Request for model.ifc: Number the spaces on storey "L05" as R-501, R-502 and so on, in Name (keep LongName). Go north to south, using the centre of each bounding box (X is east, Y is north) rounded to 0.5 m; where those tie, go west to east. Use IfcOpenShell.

First a look at what the model holds.

```python
import ifcopenshell
import ifcopenshell.util.element
import ifcopenshell.util.placement

model = ifcopenshell.open("model.ifc")
print(model.schema)
storey = next(s for s in model.by_type("IfcBuildingStorey") if s.Name == "L05")
spaces = [e for e in ifcopenshell.util.element.get_decomposition(storey) if e.is_a("IfcSpace")]
for e in sorted(spaces, key=lambda e: e.id()):
    origin = ifcopenshell.util.placement.get_local_placement(e.ObjectPlacement)[:3, 3]
    print(e.id(), e.Name, e.LongName, origin.round(2) + 0.0, sep=" | ")
```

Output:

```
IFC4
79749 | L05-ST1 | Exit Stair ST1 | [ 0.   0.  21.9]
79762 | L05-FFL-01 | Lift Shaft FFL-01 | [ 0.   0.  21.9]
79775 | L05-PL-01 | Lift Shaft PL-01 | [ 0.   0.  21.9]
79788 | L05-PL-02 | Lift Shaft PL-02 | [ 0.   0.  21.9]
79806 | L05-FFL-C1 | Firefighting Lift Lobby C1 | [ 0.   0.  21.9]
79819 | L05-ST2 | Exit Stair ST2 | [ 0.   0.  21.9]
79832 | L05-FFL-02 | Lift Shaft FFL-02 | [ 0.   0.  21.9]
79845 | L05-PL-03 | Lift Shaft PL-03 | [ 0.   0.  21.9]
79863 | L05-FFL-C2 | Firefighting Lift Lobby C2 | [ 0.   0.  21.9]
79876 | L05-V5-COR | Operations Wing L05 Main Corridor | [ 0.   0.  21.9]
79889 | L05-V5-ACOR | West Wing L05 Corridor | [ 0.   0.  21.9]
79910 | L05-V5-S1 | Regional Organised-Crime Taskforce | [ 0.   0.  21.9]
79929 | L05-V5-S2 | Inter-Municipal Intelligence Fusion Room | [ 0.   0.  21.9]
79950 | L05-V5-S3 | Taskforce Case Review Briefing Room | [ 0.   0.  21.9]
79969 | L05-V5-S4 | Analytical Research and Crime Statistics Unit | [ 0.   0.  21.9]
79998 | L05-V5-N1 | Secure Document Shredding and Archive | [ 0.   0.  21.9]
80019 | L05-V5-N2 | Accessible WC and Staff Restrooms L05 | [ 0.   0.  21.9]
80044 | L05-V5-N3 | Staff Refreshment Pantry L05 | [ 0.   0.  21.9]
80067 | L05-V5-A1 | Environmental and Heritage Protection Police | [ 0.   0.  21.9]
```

```python
import ifcopenshell
import ifcopenshell.geom
import ifcopenshell.util.element
import ifcopenshell.util.shape

model = ifcopenshell.open("model.ifc")
settings = ifcopenshell.geom.settings()
settings.set("use-world-coords", True)


def centre(element):
    shape = ifcopenshell.geom.create_shape(settings, element)
    return ifcopenshell.util.shape.get_bbox_centroid(shape.geometry)


storey = next(s for s in model.by_type("IfcBuildingStorey") if s.Name == "L05")
spaces = [e for e in ifcopenshell.util.element.get_decomposition(storey) if e.is_a("IfcSpace")]

# Insertion points can sit at a corner or the storey origin, so sort by the geometry (in metres).
centres = {e: centre(e) for e in spaces}
spaces.sort(key=lambda e: (-round(centres[e][1] / 0.5), centres[e][0]))

for i, e in enumerate(spaces, start=1):
    number = f"R-5{i:02d}"
    e.Name = number
    print(e.id(), number)

model.write("model_updated.ifc")
```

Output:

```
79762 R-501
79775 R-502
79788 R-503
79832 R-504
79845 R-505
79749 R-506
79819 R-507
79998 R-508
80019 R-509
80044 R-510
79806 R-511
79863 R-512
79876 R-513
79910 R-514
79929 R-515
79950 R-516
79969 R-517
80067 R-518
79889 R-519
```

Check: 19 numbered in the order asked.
